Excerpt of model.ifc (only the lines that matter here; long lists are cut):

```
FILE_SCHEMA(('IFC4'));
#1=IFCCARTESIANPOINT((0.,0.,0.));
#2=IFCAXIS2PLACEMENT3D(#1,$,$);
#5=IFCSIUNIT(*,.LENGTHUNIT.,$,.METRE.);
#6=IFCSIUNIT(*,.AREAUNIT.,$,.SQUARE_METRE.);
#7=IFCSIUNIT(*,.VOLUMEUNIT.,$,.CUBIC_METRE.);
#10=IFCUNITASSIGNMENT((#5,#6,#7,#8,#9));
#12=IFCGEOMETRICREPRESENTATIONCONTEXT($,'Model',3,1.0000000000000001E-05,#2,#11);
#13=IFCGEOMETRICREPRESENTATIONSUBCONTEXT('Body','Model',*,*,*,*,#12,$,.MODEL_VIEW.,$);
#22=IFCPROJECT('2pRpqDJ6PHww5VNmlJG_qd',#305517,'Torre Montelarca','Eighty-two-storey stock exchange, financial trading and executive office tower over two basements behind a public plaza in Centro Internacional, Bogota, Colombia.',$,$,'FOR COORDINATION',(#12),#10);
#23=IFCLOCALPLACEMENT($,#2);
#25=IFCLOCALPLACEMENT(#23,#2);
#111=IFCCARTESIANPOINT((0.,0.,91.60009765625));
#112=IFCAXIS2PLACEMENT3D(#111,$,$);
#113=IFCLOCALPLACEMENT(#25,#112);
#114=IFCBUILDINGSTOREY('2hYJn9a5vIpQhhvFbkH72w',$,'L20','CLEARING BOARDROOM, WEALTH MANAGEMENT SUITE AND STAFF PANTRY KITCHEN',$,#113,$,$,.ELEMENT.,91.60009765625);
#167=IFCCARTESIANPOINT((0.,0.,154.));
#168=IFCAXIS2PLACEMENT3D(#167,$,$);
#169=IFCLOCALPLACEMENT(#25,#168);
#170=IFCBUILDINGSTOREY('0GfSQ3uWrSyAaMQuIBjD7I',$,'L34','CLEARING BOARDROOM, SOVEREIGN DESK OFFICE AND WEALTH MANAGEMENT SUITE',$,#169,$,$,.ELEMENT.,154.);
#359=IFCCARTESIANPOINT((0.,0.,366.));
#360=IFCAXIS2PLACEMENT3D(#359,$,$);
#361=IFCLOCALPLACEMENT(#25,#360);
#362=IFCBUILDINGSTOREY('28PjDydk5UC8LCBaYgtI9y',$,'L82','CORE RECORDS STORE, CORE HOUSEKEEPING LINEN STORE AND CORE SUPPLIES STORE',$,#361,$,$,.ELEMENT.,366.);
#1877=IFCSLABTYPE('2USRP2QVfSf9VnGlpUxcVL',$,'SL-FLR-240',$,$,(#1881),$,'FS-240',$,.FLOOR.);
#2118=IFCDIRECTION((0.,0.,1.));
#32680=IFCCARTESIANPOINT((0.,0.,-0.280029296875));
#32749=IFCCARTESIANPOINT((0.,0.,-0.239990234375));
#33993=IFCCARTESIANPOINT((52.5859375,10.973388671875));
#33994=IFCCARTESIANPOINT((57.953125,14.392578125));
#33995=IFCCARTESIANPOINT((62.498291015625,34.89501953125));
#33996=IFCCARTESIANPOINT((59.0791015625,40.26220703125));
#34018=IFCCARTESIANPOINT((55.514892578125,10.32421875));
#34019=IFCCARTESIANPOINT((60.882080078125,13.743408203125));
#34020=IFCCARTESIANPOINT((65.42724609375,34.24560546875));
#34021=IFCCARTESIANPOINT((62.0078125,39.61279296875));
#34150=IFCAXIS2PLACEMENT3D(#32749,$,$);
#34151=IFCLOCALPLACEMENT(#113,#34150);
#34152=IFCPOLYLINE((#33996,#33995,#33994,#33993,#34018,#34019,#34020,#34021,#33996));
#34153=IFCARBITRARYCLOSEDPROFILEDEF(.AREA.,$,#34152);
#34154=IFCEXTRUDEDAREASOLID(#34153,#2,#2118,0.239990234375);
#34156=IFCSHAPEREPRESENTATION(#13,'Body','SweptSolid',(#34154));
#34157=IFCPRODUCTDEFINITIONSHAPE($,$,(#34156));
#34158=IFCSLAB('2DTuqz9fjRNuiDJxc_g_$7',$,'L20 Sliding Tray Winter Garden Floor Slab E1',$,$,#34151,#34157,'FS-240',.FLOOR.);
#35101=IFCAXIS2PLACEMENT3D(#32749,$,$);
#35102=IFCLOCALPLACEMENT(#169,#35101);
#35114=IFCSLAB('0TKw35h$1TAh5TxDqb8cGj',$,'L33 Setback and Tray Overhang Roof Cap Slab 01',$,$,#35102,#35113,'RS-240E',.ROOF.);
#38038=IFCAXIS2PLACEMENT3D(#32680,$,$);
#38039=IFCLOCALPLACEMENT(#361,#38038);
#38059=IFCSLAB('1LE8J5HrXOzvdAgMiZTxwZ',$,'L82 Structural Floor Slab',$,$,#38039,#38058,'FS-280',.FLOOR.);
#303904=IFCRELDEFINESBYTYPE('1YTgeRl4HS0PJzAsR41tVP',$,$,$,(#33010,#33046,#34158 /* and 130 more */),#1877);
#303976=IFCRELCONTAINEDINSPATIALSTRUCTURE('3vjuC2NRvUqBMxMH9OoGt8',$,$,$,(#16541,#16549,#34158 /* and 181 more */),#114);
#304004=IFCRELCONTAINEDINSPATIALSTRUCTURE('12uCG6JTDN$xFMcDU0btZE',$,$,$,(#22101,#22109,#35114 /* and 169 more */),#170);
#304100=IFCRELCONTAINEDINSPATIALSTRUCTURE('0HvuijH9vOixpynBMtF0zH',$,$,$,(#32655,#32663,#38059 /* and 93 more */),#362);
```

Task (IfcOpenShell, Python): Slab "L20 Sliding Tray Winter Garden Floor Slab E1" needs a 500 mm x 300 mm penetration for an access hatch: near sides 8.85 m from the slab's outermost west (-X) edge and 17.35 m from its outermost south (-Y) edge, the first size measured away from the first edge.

```python
import numpy as np
import ifcopenshell
import ifcopenshell.api.feature
import ifcopenshell.api.geometry
import ifcopenshell.api.root
import ifcopenshell.geom
import ifcopenshell.util.placement
import ifcopenshell.util.representation
import ifcopenshell.util.shape
import ifcopenshell.util.unit

model = ifcopenshell.open("model.ifc")
unit_scale = ifcopenshell.util.unit.calculate_unit_scale(model)
settings = ifcopenshell.geom.settings()


def volume(element):
    """Net volume in cubic metres, openings subtracted."""
    shape = ifcopenshell.geom.create_shape(settings, element)
    return ifcopenshell.util.shape.get_volume(shape.geometry)


slab = model.by_guid("2DTuqz9fjRNuiDJxc_g_$7")
before = volume(slab)

# Extent in the slab's own axes, in metres. The edges named are its -X and -Y sides.
slab_shape = ifcopenshell.geom.create_shape(settings, slab)
vertices = ifcopenshell.util.shape.get_vertices(slab_shape.geometry)
x_min, y_min, bottom = vertices.min(axis=0)
top = vertices[:, 2].max()

opening = ifcopenshell.api.root.create_entity(model, ifc_class="IfcOpeningElement", name="Access hatch opening", predefined_type="OPENING")
context = ifcopenshell.util.representation.get_context(model, "Model", "Body", "MODEL_VIEW")
width, depth = 0.5, 0.3
outline = [(0.0, 0.0), (width, 0.0), (width, depth), (0.0, depth), (0.0, 0.0)]
# Overshoot both faces by 50 mm so the cut is clean.
shape = ifcopenshell.api.geometry.add_slab_representation(
    model, context=context, depth=top - bottom + 0.1, polyline=outline
)
ifcopenshell.api.geometry.assign_representation(model, product=opening, representation=shape)

matrix = ifcopenshell.util.placement.get_local_placement(slab.ObjectPlacement)
matrix[:, 3] = matrix @ np.append(np.array([x_min + 8.85, y_min + 17.35, bottom - 0.05]) / unit_scale, 1.0)
ifcopenshell.api.geometry.edit_object_placement(model, product=opening, matrix=matrix, is_si=False)
ifcopenshell.api.feature.add_feature(model, feature=opening, element=slab)

after = volume(slab)

print(f"slab volume {before:.3f} -> {after:.3f} m3")

model.write("model_updated.ifc")
```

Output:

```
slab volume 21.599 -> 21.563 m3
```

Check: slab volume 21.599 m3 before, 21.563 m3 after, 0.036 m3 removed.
